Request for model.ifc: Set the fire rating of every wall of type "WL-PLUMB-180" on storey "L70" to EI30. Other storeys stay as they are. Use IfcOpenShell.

First a look at what the model holds.

```python
import ifcopenshell
import ifcopenshell.util.element

model = ifcopenshell.open("model.ifc")
print(model.schema)
storey = next(s for s in model.by_type("IfcBuildingStorey") if s.Name == "L70")
walls = [e for e in ifcopenshell.util.element.get_decomposition(storey) if e.is_a("IfcWall")]
seen = {}
for e in walls:
    element_type = ifcopenshell.util.element.get_type(e)
    key = (element_type.Name if element_type != e and element_type else None, ifcopenshell.util.element.get_pset(e, "Pset_WallCommon", "FireRating"))
    seen[key] = seen.get(key, 0) + 1
for (name, value), count in sorted(seen.items(), key=str):
    print(count, "x", name, "|", value)
```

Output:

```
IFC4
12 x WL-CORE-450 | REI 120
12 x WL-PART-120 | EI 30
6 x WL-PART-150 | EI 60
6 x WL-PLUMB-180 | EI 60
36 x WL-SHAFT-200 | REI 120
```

```python
import ifcopenshell
import ifcopenshell.api.pset
import ifcopenshell.util.element

model = ifcopenshell.open("model.ifc")

storey = next(s for s in model.by_type("IfcBuildingStorey") if s.Name == "L70")
walls = [e for e in ifcopenshell.util.element.get_decomposition(storey) if e.is_a("IfcWall")]

count = 0
for e in walls:
    element_type = ifcopenshell.util.element.get_type(e)
    if element_type in (None, e) or element_type.Name != "WL-PLUMB-180":
        continue
    # add_pset returns the element's existing set when there is one.
    pset = ifcopenshell.api.pset.add_pset(model, product=e, name="Pset_WallCommon")
    ifcopenshell.api.pset.edit_pset(model, pset=pset, properties={"FireRating": "EI30"})
    count += 1

print(count, "walls updated")

model.write("model-out.ifc")
```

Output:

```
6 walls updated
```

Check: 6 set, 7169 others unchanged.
